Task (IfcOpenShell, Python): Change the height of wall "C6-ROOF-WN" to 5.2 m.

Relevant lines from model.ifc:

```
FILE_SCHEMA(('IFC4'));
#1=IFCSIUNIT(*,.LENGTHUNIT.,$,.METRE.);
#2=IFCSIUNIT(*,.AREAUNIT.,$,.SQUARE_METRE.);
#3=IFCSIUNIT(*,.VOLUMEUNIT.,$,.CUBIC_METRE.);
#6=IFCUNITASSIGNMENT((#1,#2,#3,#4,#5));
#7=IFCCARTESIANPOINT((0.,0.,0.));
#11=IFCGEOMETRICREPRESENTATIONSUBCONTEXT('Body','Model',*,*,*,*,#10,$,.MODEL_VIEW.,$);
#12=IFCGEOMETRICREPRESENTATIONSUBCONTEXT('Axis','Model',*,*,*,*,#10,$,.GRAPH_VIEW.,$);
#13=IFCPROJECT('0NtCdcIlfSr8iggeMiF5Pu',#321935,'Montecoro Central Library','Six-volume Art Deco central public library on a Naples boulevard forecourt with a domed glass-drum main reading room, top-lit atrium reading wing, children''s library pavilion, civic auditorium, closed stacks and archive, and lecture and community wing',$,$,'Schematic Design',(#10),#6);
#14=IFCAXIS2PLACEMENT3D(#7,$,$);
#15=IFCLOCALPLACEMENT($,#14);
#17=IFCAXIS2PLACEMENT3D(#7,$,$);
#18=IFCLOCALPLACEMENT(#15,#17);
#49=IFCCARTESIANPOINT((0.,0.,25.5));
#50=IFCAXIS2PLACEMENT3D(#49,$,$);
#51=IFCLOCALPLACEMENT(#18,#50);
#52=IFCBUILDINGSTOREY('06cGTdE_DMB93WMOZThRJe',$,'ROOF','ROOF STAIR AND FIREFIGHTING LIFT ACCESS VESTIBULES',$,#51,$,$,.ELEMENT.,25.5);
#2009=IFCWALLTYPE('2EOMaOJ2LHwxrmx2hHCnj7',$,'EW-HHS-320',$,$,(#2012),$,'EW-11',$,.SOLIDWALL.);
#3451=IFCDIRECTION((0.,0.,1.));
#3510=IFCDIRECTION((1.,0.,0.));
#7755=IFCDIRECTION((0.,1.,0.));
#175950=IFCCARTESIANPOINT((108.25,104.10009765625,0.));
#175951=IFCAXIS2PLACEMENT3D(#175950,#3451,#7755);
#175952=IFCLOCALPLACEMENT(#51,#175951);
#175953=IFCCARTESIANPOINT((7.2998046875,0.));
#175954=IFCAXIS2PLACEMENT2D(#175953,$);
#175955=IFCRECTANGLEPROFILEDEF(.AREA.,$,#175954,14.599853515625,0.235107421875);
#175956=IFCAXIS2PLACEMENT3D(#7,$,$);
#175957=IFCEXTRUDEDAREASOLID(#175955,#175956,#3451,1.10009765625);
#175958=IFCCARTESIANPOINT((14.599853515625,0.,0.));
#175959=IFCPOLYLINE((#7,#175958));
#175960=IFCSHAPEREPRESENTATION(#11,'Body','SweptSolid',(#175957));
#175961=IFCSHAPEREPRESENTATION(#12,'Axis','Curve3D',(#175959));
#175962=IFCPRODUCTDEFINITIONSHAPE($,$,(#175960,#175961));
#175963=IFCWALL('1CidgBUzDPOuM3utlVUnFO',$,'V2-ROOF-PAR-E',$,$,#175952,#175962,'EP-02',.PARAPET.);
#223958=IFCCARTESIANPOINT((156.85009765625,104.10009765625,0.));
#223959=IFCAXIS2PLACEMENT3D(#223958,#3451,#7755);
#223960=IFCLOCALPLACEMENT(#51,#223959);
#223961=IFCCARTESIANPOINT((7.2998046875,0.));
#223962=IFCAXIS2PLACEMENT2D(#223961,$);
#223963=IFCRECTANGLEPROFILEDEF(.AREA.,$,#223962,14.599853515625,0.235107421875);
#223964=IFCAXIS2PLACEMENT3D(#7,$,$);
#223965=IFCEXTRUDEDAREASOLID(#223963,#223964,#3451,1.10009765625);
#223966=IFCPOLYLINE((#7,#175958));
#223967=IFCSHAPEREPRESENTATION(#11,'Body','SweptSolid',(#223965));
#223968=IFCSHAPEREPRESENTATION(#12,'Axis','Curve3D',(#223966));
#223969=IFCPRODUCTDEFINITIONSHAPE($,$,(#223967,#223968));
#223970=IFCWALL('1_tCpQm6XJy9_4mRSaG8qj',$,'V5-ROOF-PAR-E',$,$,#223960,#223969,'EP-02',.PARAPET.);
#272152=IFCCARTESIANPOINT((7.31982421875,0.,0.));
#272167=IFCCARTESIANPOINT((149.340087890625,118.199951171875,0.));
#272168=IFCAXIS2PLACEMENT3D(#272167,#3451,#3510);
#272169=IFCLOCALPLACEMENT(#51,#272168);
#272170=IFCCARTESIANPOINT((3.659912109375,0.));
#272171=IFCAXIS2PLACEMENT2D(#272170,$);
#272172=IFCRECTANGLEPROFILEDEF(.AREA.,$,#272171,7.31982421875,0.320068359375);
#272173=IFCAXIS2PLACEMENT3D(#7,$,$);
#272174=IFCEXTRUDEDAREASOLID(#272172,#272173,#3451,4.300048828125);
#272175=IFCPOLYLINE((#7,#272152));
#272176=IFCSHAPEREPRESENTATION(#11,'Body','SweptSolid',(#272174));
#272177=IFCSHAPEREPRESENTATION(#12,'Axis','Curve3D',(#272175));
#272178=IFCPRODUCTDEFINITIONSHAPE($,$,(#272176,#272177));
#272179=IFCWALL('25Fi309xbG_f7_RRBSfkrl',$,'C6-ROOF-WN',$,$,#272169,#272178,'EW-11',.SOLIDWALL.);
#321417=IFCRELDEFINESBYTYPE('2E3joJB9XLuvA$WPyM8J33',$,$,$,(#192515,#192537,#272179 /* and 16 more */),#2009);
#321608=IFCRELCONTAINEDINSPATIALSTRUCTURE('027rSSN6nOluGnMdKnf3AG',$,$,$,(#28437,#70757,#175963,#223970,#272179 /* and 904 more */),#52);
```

```python
import ifcopenshell
import ifcopenshell.geom
import ifcopenshell.util.representation
import ifcopenshell.util.shape
import ifcopenshell.util.unit

model = ifcopenshell.open("model.ifc")
unit_scale = ifcopenshell.util.unit.calculate_unit_scale(model)
settings = ifcopenshell.geom.settings()


def volume(element):
    """Net volume in cubic metres, openings subtracted."""
    shape = ifcopenshell.geom.create_shape(settings, element)
    return ifcopenshell.util.shape.get_volume(shape.geometry)


wall = model.by_id(272179)
before = volume(wall)

body = ifcopenshell.util.representation.get_representation(wall, "Model", "Body")
solid = body.Items[0]
old_height = solid.Depth
solid.Depth = 5.2 / unit_scale
after = volume(wall)

print(f"height {old_height:g} -> {solid.Depth:g}, volume {before:.3f} -> {after:.3f} m3")

model.write("model_rev.ifc")
```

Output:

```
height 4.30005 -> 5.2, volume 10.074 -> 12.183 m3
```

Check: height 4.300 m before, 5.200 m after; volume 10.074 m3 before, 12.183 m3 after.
